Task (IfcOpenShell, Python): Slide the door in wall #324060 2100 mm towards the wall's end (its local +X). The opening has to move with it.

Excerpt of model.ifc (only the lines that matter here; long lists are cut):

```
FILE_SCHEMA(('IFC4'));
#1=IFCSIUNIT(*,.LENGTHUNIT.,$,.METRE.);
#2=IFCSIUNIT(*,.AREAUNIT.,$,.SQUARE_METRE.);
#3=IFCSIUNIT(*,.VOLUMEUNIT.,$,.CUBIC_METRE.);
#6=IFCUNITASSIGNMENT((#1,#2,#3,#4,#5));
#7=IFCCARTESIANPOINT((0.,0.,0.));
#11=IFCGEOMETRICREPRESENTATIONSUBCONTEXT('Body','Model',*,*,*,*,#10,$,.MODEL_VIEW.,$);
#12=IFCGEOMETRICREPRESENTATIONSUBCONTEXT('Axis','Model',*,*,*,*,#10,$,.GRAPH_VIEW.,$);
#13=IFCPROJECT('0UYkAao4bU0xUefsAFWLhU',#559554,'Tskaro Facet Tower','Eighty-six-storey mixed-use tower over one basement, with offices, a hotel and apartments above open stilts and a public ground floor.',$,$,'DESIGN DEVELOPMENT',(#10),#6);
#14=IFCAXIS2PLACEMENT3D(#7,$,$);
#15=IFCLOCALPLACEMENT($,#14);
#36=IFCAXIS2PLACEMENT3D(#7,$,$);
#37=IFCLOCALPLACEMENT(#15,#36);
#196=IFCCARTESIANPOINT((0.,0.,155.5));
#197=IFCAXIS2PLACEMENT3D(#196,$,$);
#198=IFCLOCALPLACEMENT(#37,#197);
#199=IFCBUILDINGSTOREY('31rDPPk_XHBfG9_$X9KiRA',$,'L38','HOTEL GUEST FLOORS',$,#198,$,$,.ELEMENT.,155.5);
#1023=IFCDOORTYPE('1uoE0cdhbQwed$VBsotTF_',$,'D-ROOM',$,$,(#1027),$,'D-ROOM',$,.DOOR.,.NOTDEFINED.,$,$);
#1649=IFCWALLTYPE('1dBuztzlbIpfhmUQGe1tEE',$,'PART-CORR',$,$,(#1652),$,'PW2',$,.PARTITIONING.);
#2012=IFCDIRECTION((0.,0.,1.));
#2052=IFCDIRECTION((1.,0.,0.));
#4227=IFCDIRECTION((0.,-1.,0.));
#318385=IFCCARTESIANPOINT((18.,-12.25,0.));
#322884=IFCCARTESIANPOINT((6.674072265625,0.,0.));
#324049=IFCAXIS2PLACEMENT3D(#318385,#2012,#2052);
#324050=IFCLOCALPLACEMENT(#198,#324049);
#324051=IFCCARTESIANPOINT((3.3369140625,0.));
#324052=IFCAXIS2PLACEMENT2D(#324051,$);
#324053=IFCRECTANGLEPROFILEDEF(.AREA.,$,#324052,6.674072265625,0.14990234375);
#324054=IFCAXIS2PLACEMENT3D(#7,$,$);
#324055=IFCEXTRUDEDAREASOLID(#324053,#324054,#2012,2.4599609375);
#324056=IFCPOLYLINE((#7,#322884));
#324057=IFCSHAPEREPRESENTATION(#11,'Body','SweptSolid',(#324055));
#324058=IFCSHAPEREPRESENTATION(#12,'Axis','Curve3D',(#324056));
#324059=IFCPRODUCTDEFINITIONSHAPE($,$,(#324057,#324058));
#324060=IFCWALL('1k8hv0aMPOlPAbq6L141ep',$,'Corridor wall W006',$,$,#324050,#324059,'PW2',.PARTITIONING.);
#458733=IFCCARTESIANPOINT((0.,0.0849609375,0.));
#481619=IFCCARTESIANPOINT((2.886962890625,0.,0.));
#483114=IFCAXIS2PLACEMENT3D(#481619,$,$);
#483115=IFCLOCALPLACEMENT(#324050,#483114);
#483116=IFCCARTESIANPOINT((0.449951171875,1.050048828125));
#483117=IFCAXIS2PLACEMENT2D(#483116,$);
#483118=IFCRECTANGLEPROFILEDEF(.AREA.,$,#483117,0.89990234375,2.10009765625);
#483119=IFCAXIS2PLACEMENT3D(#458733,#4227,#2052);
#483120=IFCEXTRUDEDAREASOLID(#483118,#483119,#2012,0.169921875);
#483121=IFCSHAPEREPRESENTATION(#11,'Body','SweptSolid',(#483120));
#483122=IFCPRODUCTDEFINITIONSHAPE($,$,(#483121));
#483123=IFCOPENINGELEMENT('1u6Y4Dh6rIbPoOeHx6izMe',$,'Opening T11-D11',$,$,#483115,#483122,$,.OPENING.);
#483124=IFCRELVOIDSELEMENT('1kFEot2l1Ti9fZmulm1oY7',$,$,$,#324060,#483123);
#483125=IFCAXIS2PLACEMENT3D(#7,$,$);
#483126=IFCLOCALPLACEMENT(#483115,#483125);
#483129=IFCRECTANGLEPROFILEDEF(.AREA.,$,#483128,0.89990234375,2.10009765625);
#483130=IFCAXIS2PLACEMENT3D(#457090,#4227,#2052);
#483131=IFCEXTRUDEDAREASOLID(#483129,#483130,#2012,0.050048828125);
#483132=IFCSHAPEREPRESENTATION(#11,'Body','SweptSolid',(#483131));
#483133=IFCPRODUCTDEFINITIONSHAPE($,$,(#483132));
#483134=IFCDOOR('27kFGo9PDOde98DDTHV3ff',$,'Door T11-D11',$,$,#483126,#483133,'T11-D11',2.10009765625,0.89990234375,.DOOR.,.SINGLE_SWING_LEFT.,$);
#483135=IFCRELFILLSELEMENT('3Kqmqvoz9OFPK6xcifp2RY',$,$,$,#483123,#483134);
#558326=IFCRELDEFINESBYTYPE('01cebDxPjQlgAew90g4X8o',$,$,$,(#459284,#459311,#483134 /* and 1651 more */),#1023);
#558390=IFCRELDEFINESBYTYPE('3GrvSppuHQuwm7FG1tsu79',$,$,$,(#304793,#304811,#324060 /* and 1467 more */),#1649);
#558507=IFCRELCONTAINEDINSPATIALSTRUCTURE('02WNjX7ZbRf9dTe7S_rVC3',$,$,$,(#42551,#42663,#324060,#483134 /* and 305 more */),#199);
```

```python
import ifcopenshell
import ifcopenshell.api.geometry
import ifcopenshell.util.placement
import ifcopenshell.util.unit

model = ifcopenshell.open("model.ifc")
unit_scale = ifcopenshell.util.unit.calculate_unit_scale(model)

door = model.by_guid("27kFGo9PDOde98DDTHV3ff")
opening = door.FillsVoids[0].RelatingOpeningElement
wall = opening.VoidsElements[0].RelatingBuildingElement

wall_matrix = ifcopenshell.util.placement.get_local_placement(wall.ObjectPlacement)
shift = wall_matrix[:3, 0] * 2.1 / unit_scale
before = ifcopenshell.util.placement.get_local_placement(door.ObjectPlacement)[:3, 3].copy()

# The door is placed relative to its opening, so it follows when the opening moves.
matrix = ifcopenshell.util.placement.get_local_placement(opening.ObjectPlacement)
matrix[:3, 3] += shift
ifcopenshell.api.geometry.edit_object_placement(
    model, product=opening, matrix=matrix, is_si=False, should_transform_children=True
)

after = ifcopenshell.util.placement.get_local_placement(door.ObjectPlacement)[:3, 3]
print("door moved by", (after - before).round(3) + 0.0)

model.write("model_updated.ifc")
```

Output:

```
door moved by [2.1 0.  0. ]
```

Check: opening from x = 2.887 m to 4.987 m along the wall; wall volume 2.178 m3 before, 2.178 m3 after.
